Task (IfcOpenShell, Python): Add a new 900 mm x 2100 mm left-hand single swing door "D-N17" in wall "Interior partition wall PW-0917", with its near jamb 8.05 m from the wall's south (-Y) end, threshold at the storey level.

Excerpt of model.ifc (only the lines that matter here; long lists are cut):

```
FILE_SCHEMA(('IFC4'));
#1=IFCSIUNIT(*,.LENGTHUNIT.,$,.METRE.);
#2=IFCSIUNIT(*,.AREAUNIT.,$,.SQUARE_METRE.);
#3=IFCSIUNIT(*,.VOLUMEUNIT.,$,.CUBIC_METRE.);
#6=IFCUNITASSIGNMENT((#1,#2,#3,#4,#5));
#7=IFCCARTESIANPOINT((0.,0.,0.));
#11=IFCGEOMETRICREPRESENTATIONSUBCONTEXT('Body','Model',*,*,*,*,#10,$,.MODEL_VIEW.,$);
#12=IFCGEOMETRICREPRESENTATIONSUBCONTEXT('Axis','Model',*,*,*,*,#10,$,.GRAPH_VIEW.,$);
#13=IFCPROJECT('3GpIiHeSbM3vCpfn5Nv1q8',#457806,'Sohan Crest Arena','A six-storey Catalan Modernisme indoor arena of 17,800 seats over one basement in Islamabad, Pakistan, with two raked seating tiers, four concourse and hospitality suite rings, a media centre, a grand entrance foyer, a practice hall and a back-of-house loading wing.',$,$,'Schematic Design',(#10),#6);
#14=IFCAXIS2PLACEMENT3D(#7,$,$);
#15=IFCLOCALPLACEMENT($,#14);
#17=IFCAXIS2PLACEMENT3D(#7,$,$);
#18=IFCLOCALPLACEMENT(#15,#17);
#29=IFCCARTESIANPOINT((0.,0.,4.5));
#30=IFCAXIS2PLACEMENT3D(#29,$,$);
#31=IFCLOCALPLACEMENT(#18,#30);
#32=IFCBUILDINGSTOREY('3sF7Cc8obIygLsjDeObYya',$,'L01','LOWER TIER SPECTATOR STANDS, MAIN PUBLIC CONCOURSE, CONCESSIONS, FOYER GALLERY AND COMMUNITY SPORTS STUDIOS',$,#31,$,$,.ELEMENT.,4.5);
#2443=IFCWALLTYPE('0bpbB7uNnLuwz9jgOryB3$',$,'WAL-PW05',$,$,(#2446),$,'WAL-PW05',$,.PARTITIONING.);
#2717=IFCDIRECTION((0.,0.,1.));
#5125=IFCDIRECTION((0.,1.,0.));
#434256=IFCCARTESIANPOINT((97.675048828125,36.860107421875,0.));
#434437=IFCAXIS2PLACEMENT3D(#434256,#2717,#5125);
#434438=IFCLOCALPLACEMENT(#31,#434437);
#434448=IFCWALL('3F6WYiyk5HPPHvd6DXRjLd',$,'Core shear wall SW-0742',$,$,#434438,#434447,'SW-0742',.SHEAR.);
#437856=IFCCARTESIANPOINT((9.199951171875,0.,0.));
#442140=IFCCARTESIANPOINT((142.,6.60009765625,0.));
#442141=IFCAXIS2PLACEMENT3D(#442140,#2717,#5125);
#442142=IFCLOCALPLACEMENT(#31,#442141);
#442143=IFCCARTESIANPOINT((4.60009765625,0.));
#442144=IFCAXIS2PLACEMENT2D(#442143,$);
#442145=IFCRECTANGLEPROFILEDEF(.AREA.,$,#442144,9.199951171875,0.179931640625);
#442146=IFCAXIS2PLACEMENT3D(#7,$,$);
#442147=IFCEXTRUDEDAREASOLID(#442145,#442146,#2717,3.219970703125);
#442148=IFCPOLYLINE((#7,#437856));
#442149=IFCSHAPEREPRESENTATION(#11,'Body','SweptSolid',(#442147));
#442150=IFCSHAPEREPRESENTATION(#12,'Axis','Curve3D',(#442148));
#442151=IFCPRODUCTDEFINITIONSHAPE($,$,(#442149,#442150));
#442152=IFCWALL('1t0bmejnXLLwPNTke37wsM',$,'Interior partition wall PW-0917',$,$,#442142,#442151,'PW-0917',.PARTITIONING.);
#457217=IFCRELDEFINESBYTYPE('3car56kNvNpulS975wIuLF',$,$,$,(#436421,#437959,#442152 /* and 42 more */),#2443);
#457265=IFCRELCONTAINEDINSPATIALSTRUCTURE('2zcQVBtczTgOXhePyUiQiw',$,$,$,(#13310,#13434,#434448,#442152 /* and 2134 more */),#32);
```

```python
import numpy as np
import ifcopenshell
import ifcopenshell.api.feature
import ifcopenshell.api.geometry
import ifcopenshell.api.root
import ifcopenshell.api.spatial
import ifcopenshell.geom
import ifcopenshell.util.element
import ifcopenshell.util.placement
import ifcopenshell.util.representation
import ifcopenshell.util.shape
import ifcopenshell.util.unit

model = ifcopenshell.open("model.ifc")
unit_scale = ifcopenshell.util.unit.calculate_unit_scale(model)
settings = ifcopenshell.geom.settings()


def volume(element):
    """Net volume in cubic metres, openings subtracted."""
    shape = ifcopenshell.geom.create_shape(settings, element)
    return ifcopenshell.util.shape.get_volume(shape.geometry)


wall = model.by_id(442152)
storey = ifcopenshell.util.element.get_container(wall, ifc_class="IfcBuildingStorey")
context = ifcopenshell.util.representation.get_context(model, "Model", "Body", "MODEL_VIEW")
before = volume(wall)

width, height, from_end, sill = 0.9, 2.1, 8.05, 0.0  # metres

# The wall runs along its own X axis, and the end named is its -X end.
wall_shape = ifcopenshell.geom.create_shape(settings, wall)
x, y, z = ifcopenshell.util.shape.get_vertices(wall_shape.geometry).T
start = x.min() + from_end
face, thickness = float(y.min()), float(y.max() - y.min())
wall_matrix = ifcopenshell.util.placement.get_local_placement(wall.ObjectPlacement)
level = ifcopenshell.util.placement.get_local_placement(storey.ObjectPlacement)[2, 3]


def in_wall(x, y):
    """Placement at x, y metres in the wall's axes, at sill height."""
    matrix = wall_matrix.copy()
    matrix[:, 3] = wall_matrix @ np.array([x / unit_scale, y / unit_scale, 0.0, 1.0])
    matrix[2, 3] = level + sill / unit_scale
    return matrix


# Opening: a box that overshoots both wall faces by 50 mm.
opening = ifcopenshell.api.root.create_entity(model, ifc_class="IfcOpeningElement", predefined_type="OPENING")
box = ifcopenshell.api.geometry.add_wall_representation(
    model, context=context, length=width, height=height, thickness=thickness + 0.1
)
ifcopenshell.api.geometry.assign_representation(model, product=opening, representation=box)
ifcopenshell.api.geometry.edit_object_placement(model, product=opening, matrix=in_wall(start, face - 0.05), is_si=False)
ifcopenshell.api.feature.add_feature(model, feature=opening, element=wall)

door = ifcopenshell.api.root.create_entity(model, ifc_class="IfcDoor", name="D-N17", predefined_type="DOOR")
door.OverallWidth, door.OverallHeight = width / unit_scale, height / unit_scale
door.OperationType = "SINGLE_SWING_LEFT"
body = ifcopenshell.api.geometry.add_door_representation(
    model,
    context=context,
    overall_width=door.OverallWidth,
    overall_height=door.OverallHeight,
    operation_type="SINGLE_SWING_LEFT",
    lining_properties={"LiningDepth": thickness / unit_scale, "ThresholdDepth": thickness / unit_scale},
)
ifcopenshell.api.geometry.assign_representation(model, product=door, representation=body)
ifcopenshell.api.spatial.assign_container(model, products=[door], relating_structure=storey)
ifcopenshell.api.feature.add_filling(model, opening=opening, element=door)

# The lining spans the wall, so the door starts at the wall face.
ifcopenshell.api.geometry.edit_object_placement(model, product=door, matrix=in_wall(start, face), is_si=False)

after = volume(wall)

print(f"wall volume {before:.3f} -> {after:.3f} m3")

model.write("model-out.ifc")
```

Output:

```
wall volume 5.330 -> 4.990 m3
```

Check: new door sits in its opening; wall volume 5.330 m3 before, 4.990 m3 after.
